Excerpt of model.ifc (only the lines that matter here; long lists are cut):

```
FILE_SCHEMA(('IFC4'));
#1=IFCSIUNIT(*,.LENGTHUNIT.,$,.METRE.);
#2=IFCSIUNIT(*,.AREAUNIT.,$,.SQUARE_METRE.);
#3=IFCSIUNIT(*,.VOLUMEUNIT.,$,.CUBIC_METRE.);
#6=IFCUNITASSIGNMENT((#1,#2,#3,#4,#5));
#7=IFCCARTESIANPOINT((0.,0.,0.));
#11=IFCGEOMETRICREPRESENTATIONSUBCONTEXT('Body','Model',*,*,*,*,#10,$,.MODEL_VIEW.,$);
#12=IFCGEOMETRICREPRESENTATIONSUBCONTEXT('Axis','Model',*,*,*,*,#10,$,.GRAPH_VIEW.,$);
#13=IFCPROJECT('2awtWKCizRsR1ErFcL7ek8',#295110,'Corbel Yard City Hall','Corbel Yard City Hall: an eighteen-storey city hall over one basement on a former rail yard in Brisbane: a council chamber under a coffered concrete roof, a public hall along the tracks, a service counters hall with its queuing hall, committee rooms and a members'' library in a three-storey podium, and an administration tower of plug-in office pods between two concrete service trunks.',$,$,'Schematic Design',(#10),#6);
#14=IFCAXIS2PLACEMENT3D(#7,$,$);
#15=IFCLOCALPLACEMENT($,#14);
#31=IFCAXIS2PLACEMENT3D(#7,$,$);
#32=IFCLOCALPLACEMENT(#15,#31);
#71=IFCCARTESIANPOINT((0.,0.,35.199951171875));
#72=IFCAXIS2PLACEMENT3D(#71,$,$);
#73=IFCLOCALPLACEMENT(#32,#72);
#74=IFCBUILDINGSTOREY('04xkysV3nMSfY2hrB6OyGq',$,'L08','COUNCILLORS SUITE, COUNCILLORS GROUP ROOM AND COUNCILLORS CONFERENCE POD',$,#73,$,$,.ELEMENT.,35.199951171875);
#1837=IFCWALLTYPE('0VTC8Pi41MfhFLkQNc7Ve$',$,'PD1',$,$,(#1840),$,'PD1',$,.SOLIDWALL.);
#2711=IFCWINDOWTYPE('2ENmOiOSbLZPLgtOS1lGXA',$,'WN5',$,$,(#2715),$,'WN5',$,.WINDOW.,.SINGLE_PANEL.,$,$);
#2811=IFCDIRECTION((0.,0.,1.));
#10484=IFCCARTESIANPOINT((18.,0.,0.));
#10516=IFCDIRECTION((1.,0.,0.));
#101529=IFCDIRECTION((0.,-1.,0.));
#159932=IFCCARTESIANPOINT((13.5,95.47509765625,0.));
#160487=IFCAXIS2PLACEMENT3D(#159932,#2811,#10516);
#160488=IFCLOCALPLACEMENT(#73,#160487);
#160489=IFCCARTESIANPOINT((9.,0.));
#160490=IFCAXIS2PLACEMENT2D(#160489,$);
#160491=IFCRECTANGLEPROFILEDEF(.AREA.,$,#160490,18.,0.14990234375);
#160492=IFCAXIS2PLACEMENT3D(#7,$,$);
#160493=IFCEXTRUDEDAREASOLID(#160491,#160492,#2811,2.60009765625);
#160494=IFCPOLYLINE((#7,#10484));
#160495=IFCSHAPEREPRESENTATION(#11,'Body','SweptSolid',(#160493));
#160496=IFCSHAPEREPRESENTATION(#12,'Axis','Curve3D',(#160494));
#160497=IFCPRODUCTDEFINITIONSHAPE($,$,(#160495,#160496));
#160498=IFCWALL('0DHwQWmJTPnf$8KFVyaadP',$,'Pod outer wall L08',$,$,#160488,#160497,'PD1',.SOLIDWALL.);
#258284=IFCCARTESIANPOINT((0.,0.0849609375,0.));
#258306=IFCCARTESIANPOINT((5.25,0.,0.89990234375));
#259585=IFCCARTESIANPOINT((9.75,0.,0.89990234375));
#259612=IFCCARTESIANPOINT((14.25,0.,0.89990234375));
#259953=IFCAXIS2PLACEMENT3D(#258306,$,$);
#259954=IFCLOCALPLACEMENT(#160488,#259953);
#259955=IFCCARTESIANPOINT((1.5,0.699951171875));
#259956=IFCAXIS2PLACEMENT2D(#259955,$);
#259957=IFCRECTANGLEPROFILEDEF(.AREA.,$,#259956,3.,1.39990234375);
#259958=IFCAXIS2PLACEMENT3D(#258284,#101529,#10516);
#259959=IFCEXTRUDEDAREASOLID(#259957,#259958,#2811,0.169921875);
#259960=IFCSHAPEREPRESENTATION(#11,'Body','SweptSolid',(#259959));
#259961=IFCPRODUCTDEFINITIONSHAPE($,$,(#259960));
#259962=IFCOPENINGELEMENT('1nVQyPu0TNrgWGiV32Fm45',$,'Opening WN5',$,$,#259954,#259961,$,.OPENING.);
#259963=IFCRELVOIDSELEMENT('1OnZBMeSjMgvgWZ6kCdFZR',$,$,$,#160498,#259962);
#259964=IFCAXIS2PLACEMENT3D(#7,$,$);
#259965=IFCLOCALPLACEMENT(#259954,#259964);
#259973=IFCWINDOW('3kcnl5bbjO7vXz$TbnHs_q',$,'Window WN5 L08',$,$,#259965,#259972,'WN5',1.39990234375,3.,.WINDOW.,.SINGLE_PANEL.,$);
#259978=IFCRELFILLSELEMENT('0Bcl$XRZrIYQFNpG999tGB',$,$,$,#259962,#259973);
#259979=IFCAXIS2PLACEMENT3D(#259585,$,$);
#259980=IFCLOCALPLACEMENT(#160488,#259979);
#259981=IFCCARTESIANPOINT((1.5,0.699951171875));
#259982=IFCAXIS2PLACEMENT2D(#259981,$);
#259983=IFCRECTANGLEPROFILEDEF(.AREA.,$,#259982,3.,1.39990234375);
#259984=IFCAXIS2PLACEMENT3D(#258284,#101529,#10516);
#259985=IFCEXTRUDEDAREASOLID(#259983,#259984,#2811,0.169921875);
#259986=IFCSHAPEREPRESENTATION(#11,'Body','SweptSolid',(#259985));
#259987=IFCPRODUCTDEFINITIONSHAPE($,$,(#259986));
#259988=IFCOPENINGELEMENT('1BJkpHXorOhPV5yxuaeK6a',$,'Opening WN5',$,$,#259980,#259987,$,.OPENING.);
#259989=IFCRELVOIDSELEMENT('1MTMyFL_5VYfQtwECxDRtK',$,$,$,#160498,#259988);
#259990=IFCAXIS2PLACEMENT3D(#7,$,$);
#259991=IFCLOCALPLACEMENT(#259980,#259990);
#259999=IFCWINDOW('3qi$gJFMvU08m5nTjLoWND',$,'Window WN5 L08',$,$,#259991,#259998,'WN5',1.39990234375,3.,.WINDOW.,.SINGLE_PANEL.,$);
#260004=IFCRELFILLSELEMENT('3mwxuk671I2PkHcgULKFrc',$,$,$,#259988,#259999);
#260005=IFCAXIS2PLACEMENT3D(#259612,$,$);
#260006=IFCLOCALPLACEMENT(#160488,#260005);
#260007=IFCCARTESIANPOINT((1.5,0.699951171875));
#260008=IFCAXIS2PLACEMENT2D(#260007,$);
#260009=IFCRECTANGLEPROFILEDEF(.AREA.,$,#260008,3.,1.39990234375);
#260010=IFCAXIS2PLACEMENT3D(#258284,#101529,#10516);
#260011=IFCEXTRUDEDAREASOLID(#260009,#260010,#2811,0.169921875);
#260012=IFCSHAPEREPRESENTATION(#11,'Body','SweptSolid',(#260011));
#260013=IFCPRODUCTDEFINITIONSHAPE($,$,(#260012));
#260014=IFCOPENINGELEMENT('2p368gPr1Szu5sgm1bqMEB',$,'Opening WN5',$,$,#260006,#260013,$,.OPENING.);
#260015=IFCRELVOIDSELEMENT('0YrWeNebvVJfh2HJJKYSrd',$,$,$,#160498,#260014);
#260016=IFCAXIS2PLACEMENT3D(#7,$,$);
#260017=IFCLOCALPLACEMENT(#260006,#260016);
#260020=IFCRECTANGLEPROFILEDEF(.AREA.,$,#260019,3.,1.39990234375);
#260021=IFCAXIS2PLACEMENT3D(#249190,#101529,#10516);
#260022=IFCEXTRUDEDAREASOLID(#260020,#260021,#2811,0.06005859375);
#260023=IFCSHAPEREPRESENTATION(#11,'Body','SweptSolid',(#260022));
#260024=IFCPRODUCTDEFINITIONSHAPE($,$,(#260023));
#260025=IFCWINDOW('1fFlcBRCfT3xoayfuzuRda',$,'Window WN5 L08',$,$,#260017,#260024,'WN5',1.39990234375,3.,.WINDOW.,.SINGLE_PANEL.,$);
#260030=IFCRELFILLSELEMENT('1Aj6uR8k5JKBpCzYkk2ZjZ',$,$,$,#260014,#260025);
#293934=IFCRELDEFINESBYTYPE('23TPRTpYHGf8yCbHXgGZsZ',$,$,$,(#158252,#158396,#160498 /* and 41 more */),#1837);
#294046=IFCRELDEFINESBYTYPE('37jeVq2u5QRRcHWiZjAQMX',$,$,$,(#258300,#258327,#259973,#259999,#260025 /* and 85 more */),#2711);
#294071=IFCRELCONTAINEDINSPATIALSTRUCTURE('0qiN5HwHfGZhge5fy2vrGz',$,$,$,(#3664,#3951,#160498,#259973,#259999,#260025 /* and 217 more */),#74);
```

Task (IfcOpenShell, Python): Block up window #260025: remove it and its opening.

```python
import ifcopenshell
import ifcopenshell.api.feature
import ifcopenshell.api.root
import ifcopenshell.geom
import ifcopenshell.util.shape

model = ifcopenshell.open("model.ifc")
settings = ifcopenshell.geom.settings()


def volume(element):
    """Net volume in cubic metres, openings subtracted."""
    shape = ifcopenshell.geom.create_shape(settings, element)
    return ifcopenshell.util.shape.get_volume(shape.geometry)


window = model.by_guid("1fFlcBRCfT3xoayfuzuRda")
opening = window.FillsVoids[0].RelatingOpeningElement
wall = opening.VoidsElements[0].RelatingBuildingElement
before = volume(wall)

ifcopenshell.api.root.remove_product(model, product=window)
ifcopenshell.api.feature.remove_feature(model, feature=opening)

after = volume(wall)

print(f"wall volume {before:.3f} -> {after:.3f} m3")

model.write("model_updated.ifc")
```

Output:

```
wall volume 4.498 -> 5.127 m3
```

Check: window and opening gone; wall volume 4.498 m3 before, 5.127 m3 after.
